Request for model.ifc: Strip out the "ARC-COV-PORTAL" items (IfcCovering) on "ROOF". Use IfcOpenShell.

First a look at what the model holds.

```python
import ifcopenshell
import ifcopenshell.util.element

model = ifcopenshell.open("model.ifc")
print(model.schema)
storey = next(s for s in model.by_type("IfcBuildingStorey") if s.Name == "ROOF")
coverings = [e for e in ifcopenshell.util.element.get_decomposition(storey) if e.is_a("IfcCovering")]
seen = {}
for e in coverings:
    element_type = ifcopenshell.util.element.get_type(e)
    name = element_type.Name if element_type not in (None, e) else None
    seen[name] = seen.get(name, 0) + 1
for name, count in sorted(seen.items(), key=str):
    print(count, "x", name)
```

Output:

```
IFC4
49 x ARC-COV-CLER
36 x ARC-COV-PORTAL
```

```python
import ifcopenshell
import ifcopenshell.api.root
import ifcopenshell.util.element

model = ifcopenshell.open("model.ifc")

storey = next(s for s in model.by_type("IfcBuildingStorey") if s.Name == "ROOF")
coverings = [e for e in ifcopenshell.util.element.get_decomposition(storey) if e.is_a("IfcCovering")]
targets = [e for e in coverings if (t := ifcopenshell.util.element.get_type(e)) not in (None, e) and t.Name == "ARC-COV-PORTAL"]

for e in targets:
    ifcopenshell.api.root.remove_product(model, product=e)
print(len(targets), "removed")

model.write("model_v2.ifc")
```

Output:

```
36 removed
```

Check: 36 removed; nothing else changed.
